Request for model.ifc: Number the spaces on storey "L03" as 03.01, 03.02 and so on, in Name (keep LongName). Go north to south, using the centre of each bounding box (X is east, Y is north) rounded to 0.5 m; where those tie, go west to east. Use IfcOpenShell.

First a look at what the model holds.

```python
import ifcopenshell
import ifcopenshell.util.element
import ifcopenshell.util.placement

model = ifcopenshell.open("model.ifc")
print(model.schema)
storey = next(s for s in model.by_type("IfcBuildingStorey") if s.Name == "L03")
spaces = [e for e in ifcopenshell.util.element.get_decomposition(storey) if e.is_a("IfcSpace")]
for e in sorted(spaces, key=lambda e: e.id()):
    origin = ifcopenshell.util.placement.get_local_placement(e.ObjectPlacement)[:3, 3]
    print(e.id(), e.Name, e.LongName, origin.round(2) + 0.0, sep=" | ")
```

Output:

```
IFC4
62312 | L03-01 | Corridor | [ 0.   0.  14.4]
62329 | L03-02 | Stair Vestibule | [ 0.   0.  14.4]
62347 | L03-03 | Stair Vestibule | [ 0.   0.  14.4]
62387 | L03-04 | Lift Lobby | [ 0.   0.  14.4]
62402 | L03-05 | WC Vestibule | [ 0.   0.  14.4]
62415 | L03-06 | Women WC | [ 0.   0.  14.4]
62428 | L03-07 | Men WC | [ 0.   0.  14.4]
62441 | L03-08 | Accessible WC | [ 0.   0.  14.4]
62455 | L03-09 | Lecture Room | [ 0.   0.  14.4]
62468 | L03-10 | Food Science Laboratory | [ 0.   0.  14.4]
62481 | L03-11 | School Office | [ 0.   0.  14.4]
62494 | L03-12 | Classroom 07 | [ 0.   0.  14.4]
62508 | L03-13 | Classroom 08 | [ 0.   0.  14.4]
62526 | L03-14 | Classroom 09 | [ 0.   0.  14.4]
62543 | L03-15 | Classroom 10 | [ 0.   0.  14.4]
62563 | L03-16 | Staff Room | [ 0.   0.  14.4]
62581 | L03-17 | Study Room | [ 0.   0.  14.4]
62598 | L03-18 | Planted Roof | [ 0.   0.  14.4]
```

```python
import ifcopenshell
import ifcopenshell.geom
import ifcopenshell.util.element
import ifcopenshell.util.shape

model = ifcopenshell.open("model.ifc")
settings = ifcopenshell.geom.settings()
settings.set("use-world-coords", True)


def centre(element):
    shape = ifcopenshell.geom.create_shape(settings, element)
    return ifcopenshell.util.shape.get_bbox_centroid(shape.geometry)


storey = next(s for s in model.by_type("IfcBuildingStorey") if s.Name == "L03")
spaces = [e for e in ifcopenshell.util.element.get_decomposition(storey) if e.is_a("IfcSpace")]

# Insertion points can sit at a corner or the storey origin, so sort by the geometry (in metres).
centres = {e: centre(e) for e in spaces}
spaces.sort(key=lambda e: (-round(centres[e][1] / 0.5), centres[e][0]))

for i, e in enumerate(spaces, start=1):
    number = f"03.{i:02d}"
    e.Name = number
    print(e.id(), number)

model.write("model_rev.ifc")
```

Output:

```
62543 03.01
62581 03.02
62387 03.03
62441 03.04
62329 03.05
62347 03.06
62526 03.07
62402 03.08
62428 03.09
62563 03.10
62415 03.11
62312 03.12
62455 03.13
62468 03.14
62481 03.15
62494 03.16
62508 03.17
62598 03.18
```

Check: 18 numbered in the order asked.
